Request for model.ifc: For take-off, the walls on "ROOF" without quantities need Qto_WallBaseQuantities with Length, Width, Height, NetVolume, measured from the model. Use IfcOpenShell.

First a look at what the model holds.

```python
import ifcopenshell
import ifcopenshell.util.element
import ifcopenshell.util.unit

model = ifcopenshell.open("model.ifc")
print(model.schema)
for unit_type in ("LENGTHUNIT", "AREAUNIT", "VOLUMEUNIT"):
    print(unit_type, ifcopenshell.util.unit.calculate_unit_scale(model, unit_type))
storey = next(s for s in model.by_type("IfcBuildingStorey") if s.Name == "ROOF")
walls = [e for e in ifcopenshell.util.element.get_decomposition(storey) if e.is_a("IfcWall")]
for e in sorted(walls, key=lambda e: e.id()):
    print(e.id(), e.is_a(), e.Name, list(ifcopenshell.util.element.get_psets(e, qtos_only=True)), sep=" | ")
```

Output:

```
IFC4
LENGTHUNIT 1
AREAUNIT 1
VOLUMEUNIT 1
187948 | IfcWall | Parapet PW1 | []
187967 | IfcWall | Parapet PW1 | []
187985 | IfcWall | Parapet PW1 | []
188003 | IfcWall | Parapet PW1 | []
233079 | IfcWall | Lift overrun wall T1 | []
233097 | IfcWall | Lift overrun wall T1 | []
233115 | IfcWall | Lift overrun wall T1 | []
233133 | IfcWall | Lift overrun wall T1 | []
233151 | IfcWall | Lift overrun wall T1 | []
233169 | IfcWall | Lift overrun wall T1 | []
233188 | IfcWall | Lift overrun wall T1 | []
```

```python
import ifcopenshell
import ifcopenshell.api.pset
import ifcopenshell.geom
import ifcopenshell.util.element
import ifcopenshell.util.shape
import ifcopenshell.util.unit

model = ifcopenshell.open("model.ifc")
unit_scale = ifcopenshell.util.unit.calculate_unit_scale(model)
volume_scale = ifcopenshell.util.unit.calculate_unit_scale(model, "VOLUMEUNIT")
settings = ifcopenshell.geom.settings()

storey = next(s for s in model.by_type("IfcBuildingStorey") if s.Name == "ROOF")
walls = [e for e in ifcopenshell.util.element.get_decomposition(storey) if e.is_a("IfcWall")]

for e in sorted(walls, key=lambda e: e.id()):
    if ifcopenshell.util.element.get_psets(e, qtos_only=True, should_inherit=False):
        continue
    # Geometry comes back in metres, in the element's own axes.
    shape = ifcopenshell.geom.create_shape(settings, e)
    values = {
        "Length": ifcopenshell.util.shape.get_x(shape.geometry) / unit_scale,
        "Width": ifcopenshell.util.shape.get_y(shape.geometry) / unit_scale,
        "Height": ifcopenshell.util.shape.get_z(shape.geometry) / unit_scale,
        "NetVolume": ifcopenshell.util.shape.get_volume(shape.geometry) / volume_scale,
    }
    qto = ifcopenshell.api.pset.add_qto(model, product=e, name="Qto_WallBaseQuantities")
    ifcopenshell.api.pset.edit_qto(model, qto=qto, properties=values)
    print(e.id(), {k: round(v, 3) for k, v in values.items()})

model.write("model-out.ifc")
```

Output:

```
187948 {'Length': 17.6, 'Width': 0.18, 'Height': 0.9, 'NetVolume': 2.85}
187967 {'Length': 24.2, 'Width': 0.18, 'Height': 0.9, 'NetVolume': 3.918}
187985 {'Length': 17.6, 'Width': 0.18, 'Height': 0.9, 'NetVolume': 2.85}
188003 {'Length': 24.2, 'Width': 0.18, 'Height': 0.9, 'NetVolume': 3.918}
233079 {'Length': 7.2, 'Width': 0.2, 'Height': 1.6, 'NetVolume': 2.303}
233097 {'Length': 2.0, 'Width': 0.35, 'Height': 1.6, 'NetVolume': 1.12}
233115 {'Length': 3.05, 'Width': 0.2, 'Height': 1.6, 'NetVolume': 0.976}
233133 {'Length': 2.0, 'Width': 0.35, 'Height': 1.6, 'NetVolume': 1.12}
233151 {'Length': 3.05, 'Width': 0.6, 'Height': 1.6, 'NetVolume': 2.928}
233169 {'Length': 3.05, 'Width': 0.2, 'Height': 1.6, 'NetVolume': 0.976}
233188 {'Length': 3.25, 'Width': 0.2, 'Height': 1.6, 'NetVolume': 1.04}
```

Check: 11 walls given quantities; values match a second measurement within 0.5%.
